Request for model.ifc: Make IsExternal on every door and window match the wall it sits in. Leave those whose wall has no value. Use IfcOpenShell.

First a look at what the model holds.

```python
import ifcopenshell
import ifcopenshell.util.element

model = ifcopenshell.open("model.ifc")
print(model.schema)
seen = {}
for e in model.by_type("IfcDoor") + model.by_type("IfcWindow"):
    if not e.FillsVoids:
        continue
    host = e.FillsVoids[0].RelatingOpeningElement.VoidsElements[0].RelatingBuildingElement
    own = ifcopenshell.util.element.get_pset(e, f"Pset_{e.is_a()[3:].removesuffix('StandardCase')}Common", "IsExternal")
    wall = ifcopenshell.util.element.get_pset(host, "Pset_WallCommon", "IsExternal")
    seen[e.is_a(), own, wall] = seen.get((e.is_a(), own, wall), 0) + 1
for (cls, own, wall), count in sorted(seen.items(), key=str):
    print(count, cls, "IsExternal:", own, "| host wall:", wall)
```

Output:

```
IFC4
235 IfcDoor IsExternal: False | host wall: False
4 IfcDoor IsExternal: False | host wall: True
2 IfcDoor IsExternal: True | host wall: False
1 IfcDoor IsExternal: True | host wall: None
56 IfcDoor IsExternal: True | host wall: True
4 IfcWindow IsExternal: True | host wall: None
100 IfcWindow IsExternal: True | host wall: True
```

```python
import ifcopenshell
import ifcopenshell.api.pset
import ifcopenshell.util.element

model = ifcopenshell.open("model.ifc")

count = 0
for ifc_class, pset_name in (("IfcDoor", "Pset_DoorCommon"), ("IfcWindow", "Pset_WindowCommon")):
    for e in model.by_type(ifc_class):
        if not e.FillsVoids:
            continue
        host = e.FillsVoids[0].RelatingOpeningElement.VoidsElements[0].RelatingBuildingElement
        external = ifcopenshell.util.element.get_pset(host, "Pset_WallCommon", "IsExternal")
        if external is None or ifcopenshell.util.element.get_pset(e, pset_name, "IsExternal") == external:
            continue
        pset = ifcopenshell.api.pset.add_pset(model, product=e, name=pset_name)
        ifcopenshell.api.pset.edit_pset(model, pset=pset, properties={"IsExternal": external})
        count += 1

print(count, "updated")

model.write("model_updated.ifc")
```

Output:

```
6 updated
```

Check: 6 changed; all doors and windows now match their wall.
